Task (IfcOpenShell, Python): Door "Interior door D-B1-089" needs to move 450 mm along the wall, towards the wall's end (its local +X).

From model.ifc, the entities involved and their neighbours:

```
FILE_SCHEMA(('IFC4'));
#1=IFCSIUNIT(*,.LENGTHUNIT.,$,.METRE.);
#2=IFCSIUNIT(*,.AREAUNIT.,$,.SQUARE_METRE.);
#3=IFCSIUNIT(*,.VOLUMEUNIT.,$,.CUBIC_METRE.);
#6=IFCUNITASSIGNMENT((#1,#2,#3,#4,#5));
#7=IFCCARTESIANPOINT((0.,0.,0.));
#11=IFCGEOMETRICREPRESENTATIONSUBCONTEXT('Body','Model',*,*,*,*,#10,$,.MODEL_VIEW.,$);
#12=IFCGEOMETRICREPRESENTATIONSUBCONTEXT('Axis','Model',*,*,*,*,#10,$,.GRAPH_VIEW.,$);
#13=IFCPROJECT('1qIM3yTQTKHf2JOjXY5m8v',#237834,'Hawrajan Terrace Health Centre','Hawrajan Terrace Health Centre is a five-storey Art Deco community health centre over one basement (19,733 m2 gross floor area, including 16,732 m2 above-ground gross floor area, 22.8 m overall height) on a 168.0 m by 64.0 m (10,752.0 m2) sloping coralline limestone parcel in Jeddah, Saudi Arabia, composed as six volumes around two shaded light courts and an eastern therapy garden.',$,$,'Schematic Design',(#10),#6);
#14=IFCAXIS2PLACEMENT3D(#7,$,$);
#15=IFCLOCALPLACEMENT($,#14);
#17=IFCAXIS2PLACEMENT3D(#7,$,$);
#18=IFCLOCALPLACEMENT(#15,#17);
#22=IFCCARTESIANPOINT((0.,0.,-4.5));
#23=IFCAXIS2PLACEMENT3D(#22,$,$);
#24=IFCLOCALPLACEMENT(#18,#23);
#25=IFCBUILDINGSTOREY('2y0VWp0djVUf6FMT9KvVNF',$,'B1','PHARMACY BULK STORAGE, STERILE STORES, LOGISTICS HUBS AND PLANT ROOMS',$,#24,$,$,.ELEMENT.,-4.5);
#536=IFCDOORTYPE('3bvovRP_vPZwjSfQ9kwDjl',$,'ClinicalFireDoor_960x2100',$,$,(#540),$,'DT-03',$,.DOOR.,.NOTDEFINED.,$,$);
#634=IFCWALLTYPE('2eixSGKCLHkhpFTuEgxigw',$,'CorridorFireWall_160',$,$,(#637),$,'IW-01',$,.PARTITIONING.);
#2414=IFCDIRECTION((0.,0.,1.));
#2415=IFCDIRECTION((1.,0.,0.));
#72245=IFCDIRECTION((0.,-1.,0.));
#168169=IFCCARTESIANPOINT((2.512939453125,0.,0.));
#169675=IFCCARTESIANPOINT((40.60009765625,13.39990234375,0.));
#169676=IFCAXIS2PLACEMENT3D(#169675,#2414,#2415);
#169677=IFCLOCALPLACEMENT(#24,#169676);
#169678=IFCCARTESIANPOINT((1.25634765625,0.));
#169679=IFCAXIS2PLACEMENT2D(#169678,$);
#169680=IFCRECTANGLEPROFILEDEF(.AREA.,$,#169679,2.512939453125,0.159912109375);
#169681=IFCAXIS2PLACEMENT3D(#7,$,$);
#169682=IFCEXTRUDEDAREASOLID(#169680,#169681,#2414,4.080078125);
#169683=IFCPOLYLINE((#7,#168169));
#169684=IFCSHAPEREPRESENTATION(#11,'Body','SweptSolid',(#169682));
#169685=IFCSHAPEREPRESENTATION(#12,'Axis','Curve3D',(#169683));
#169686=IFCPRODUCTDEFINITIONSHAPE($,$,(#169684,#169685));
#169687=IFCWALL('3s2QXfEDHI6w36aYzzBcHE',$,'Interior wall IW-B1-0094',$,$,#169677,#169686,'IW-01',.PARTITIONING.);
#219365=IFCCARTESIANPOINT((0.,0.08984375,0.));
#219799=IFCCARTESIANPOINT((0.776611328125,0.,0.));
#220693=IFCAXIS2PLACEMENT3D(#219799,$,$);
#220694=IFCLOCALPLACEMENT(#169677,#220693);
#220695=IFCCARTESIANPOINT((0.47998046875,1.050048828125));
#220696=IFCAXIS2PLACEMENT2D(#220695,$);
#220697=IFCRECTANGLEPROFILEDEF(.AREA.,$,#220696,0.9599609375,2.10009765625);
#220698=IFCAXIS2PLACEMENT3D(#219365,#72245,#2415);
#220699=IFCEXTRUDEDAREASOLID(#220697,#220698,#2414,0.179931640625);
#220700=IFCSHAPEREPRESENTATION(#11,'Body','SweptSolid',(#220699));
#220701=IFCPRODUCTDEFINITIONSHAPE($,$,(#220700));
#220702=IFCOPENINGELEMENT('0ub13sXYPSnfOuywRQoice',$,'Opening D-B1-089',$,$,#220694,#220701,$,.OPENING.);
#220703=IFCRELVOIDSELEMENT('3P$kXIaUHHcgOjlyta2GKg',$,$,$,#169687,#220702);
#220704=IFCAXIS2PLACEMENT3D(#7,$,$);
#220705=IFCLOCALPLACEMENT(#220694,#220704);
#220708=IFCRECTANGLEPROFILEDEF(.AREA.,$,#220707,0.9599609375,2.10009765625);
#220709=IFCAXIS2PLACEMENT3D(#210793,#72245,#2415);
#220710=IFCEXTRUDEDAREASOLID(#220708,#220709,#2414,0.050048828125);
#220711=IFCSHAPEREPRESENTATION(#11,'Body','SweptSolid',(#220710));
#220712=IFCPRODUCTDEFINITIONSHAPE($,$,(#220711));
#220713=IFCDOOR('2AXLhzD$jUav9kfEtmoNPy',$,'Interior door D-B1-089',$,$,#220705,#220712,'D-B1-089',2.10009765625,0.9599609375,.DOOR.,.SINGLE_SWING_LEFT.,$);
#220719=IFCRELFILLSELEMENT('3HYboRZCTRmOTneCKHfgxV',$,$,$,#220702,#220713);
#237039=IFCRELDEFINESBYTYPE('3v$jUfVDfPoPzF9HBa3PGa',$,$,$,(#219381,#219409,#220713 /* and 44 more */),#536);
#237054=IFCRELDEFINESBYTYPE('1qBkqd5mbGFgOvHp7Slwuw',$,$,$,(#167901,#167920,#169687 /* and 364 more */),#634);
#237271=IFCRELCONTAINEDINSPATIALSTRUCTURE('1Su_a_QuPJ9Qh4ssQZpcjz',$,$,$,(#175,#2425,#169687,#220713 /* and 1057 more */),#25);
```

```python
import ifcopenshell
import ifcopenshell.api.geometry
import ifcopenshell.util.placement
import ifcopenshell.util.unit

model = ifcopenshell.open("model.ifc")
unit_scale = ifcopenshell.util.unit.calculate_unit_scale(model)

door = model.by_guid("2AXLhzD$jUav9kfEtmoNPy")
opening = door.FillsVoids[0].RelatingOpeningElement
wall = opening.VoidsElements[0].RelatingBuildingElement

wall_matrix = ifcopenshell.util.placement.get_local_placement(wall.ObjectPlacement)
shift = wall_matrix[:3, 0] * 0.45 / unit_scale
before = ifcopenshell.util.placement.get_local_placement(door.ObjectPlacement)[:3, 3].copy()

# The door is placed relative to its opening, so it follows when the opening moves.
matrix = ifcopenshell.util.placement.get_local_placement(opening.ObjectPlacement)
matrix[:3, 3] += shift
ifcopenshell.api.geometry.edit_object_placement(
    model, product=opening, matrix=matrix, is_si=False, should_transform_children=True
)

after = ifcopenshell.util.placement.get_local_placement(door.ObjectPlacement)[:3, 3]
print("door moved by", (after - before).round(3) + 0.0)

model.write("model_v2.ifc")
```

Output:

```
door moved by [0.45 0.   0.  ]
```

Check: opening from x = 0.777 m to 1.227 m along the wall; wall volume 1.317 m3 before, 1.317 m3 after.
